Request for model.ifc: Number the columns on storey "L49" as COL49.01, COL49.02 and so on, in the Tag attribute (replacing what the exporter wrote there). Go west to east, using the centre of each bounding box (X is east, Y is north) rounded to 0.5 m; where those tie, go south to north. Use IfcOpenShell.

First a look at what the model holds.

```python
import ifcopenshell
import ifcopenshell.util.element
import ifcopenshell.util.placement

model = ifcopenshell.open("model.ifc")
print(model.schema)
storey = next(s for s in model.by_type("IfcBuildingStorey") if s.Name == "L49")
columns = [e for e in ifcopenshell.util.element.get_decomposition(storey) if e.is_a("IfcColumn")]
for e in sorted(columns, key=lambda e: e.id()):
    origin = ifcopenshell.util.placement.get_local_placement(e.ObjectPlacement)[:3, 3]
    print(e.id(), e.Tag, e.Name, origin.round(2) + 0.0, sep=" | ")
```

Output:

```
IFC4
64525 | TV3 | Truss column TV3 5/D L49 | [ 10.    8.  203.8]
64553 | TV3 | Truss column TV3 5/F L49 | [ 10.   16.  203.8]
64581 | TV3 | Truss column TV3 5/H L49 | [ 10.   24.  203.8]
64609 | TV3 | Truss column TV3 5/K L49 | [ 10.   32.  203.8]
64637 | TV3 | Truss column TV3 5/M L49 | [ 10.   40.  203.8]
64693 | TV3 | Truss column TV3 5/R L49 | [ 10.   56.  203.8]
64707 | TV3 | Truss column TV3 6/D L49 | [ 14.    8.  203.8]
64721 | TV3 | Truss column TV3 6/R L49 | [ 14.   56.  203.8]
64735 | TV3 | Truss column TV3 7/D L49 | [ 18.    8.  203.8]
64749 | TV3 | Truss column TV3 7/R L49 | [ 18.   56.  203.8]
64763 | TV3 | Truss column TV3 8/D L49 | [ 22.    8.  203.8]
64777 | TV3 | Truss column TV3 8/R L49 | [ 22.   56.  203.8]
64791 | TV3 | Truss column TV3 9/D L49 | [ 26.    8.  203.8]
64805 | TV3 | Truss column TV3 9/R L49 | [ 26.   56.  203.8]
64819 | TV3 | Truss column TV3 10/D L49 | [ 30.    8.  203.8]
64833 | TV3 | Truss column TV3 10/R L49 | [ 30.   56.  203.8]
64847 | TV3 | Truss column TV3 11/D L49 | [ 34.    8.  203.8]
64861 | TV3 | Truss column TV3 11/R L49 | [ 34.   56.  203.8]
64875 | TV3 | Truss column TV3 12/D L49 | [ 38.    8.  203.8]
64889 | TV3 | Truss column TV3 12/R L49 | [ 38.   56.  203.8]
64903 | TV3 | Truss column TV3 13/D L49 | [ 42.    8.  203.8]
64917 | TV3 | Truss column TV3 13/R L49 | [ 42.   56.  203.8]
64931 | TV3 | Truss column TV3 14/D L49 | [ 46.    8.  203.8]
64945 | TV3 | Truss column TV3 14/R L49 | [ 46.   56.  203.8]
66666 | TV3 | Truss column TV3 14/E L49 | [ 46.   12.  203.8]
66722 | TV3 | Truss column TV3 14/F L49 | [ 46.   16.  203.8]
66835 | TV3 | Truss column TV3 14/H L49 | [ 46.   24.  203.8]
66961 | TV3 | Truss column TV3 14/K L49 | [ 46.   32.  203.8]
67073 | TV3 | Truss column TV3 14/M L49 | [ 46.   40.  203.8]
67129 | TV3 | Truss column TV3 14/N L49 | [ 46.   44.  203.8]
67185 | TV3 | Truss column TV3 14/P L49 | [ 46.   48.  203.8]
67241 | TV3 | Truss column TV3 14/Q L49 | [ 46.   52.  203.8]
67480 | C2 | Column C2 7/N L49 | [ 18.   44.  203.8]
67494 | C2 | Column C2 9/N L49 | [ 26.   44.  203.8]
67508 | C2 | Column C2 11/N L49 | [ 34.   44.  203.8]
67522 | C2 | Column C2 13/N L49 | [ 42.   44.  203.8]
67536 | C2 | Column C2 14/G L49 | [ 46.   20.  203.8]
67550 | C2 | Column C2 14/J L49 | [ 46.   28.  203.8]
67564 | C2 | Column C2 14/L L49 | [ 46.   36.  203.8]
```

```python
import ifcopenshell
import ifcopenshell.geom
import ifcopenshell.util.element
import ifcopenshell.util.shape

model = ifcopenshell.open("model.ifc")
settings = ifcopenshell.geom.settings()
settings.set("use-world-coords", True)


def centre(element):
    shape = ifcopenshell.geom.create_shape(settings, element)
    return ifcopenshell.util.shape.get_bbox_centroid(shape.geometry)


storey = next(s for s in model.by_type("IfcBuildingStorey") if s.Name == "L49")
columns = [e for e in ifcopenshell.util.element.get_decomposition(storey) if e.is_a("IfcColumn")]

# Insertion points can sit at a corner or the storey origin, so sort by the geometry (in metres).
centres = {e: centre(e) for e in columns}
columns.sort(key=lambda e: (round(centres[e][0] / 0.5), centres[e][1]))

for i, e in enumerate(columns, start=1):
    number = f"COL49.{i:02d}"
    e.Tag = number
    print(e.id(), number)

model.write("model_edited.ifc")
```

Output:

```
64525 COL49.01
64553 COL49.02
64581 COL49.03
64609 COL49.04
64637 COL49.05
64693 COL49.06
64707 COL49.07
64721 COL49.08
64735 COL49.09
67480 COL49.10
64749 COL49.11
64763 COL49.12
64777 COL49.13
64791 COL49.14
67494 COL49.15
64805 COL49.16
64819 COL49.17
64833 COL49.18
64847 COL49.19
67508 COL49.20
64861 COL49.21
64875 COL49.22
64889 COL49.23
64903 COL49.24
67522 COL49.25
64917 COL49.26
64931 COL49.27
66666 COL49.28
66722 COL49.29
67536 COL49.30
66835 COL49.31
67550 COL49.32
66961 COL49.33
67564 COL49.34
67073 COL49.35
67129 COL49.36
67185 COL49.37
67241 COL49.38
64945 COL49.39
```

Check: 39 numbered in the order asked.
